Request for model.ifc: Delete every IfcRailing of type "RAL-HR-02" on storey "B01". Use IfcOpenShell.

First a look at what the model holds.

```python
import ifcopenshell
import ifcopenshell.util.element

model = ifcopenshell.open("model.ifc")
print(model.schema)
storey = next(s for s in model.by_type("IfcBuildingStorey") if s.Name == "B01")
railings = [e for e in ifcopenshell.util.element.get_decomposition(storey) if e.is_a("IfcRailing")]
seen = {}
for e in railings:
    element_type = ifcopenshell.util.element.get_type(e)
    name = element_type.Name if element_type not in (None, e) else None
    seen[name] = seen.get(name, 0) + 1
for name, count in sorted(seen.items(), key=str):
    print(count, "x", name)
```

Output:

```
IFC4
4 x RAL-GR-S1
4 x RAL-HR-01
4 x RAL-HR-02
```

```python
import ifcopenshell
import ifcopenshell.api.root
import ifcopenshell.util.element

model = ifcopenshell.open("model.ifc")

storey = next(s for s in model.by_type("IfcBuildingStorey") if s.Name == "B01")
railings = [e for e in ifcopenshell.util.element.get_decomposition(storey) if e.is_a("IfcRailing")]
targets = [e for e in railings if (t := ifcopenshell.util.element.get_type(e)) not in (None, e) and t.Name == "RAL-HR-02"]

for e in targets:
    ifcopenshell.api.root.remove_product(model, product=e)
print(len(targets), "removed")

model.write("model-out.ifc")
```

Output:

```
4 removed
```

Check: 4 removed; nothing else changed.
